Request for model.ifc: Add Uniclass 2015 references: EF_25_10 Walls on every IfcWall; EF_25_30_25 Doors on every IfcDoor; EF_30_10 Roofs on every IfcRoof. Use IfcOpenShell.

First a look at what the model holds.

```python
import ifcopenshell

model = ifcopenshell.open("model.ifc")
print(model.schema)
print("classifications:", [c.Name for c in model.by_type("IfcClassification")])
for ifc_class in ("IfcDoor", "IfcRoof", "IfcStair", "IfcWall", "IfcWindow"):
    print(ifc_class, len(model.by_type(ifc_class)))
```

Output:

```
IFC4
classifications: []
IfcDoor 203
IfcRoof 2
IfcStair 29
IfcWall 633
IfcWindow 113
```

```python
import ifcopenshell
import ifcopenshell.api.classification

model = ifcopenshell.open("model.ifc")

system = ifcopenshell.api.classification.add_classification(model, classification="Uniclass 2015")

codes = {
    "IfcWall": ("EF_25_10", "Walls"),
    "IfcDoor": ("EF_25_30_25", "Doors"),
    "IfcRoof": ("EF_30_10", "Roofs"),
}
for ifc_class, (code, name) in codes.items():
    products = model.by_type(ifc_class)
    ifcopenshell.api.classification.add_reference(
        model, products=products, classification=system, identification=code, name=name
    )
    print(code, len(products))

model.write("model-out.ifc")
```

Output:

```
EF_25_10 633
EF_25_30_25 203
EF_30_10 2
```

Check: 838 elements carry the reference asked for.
